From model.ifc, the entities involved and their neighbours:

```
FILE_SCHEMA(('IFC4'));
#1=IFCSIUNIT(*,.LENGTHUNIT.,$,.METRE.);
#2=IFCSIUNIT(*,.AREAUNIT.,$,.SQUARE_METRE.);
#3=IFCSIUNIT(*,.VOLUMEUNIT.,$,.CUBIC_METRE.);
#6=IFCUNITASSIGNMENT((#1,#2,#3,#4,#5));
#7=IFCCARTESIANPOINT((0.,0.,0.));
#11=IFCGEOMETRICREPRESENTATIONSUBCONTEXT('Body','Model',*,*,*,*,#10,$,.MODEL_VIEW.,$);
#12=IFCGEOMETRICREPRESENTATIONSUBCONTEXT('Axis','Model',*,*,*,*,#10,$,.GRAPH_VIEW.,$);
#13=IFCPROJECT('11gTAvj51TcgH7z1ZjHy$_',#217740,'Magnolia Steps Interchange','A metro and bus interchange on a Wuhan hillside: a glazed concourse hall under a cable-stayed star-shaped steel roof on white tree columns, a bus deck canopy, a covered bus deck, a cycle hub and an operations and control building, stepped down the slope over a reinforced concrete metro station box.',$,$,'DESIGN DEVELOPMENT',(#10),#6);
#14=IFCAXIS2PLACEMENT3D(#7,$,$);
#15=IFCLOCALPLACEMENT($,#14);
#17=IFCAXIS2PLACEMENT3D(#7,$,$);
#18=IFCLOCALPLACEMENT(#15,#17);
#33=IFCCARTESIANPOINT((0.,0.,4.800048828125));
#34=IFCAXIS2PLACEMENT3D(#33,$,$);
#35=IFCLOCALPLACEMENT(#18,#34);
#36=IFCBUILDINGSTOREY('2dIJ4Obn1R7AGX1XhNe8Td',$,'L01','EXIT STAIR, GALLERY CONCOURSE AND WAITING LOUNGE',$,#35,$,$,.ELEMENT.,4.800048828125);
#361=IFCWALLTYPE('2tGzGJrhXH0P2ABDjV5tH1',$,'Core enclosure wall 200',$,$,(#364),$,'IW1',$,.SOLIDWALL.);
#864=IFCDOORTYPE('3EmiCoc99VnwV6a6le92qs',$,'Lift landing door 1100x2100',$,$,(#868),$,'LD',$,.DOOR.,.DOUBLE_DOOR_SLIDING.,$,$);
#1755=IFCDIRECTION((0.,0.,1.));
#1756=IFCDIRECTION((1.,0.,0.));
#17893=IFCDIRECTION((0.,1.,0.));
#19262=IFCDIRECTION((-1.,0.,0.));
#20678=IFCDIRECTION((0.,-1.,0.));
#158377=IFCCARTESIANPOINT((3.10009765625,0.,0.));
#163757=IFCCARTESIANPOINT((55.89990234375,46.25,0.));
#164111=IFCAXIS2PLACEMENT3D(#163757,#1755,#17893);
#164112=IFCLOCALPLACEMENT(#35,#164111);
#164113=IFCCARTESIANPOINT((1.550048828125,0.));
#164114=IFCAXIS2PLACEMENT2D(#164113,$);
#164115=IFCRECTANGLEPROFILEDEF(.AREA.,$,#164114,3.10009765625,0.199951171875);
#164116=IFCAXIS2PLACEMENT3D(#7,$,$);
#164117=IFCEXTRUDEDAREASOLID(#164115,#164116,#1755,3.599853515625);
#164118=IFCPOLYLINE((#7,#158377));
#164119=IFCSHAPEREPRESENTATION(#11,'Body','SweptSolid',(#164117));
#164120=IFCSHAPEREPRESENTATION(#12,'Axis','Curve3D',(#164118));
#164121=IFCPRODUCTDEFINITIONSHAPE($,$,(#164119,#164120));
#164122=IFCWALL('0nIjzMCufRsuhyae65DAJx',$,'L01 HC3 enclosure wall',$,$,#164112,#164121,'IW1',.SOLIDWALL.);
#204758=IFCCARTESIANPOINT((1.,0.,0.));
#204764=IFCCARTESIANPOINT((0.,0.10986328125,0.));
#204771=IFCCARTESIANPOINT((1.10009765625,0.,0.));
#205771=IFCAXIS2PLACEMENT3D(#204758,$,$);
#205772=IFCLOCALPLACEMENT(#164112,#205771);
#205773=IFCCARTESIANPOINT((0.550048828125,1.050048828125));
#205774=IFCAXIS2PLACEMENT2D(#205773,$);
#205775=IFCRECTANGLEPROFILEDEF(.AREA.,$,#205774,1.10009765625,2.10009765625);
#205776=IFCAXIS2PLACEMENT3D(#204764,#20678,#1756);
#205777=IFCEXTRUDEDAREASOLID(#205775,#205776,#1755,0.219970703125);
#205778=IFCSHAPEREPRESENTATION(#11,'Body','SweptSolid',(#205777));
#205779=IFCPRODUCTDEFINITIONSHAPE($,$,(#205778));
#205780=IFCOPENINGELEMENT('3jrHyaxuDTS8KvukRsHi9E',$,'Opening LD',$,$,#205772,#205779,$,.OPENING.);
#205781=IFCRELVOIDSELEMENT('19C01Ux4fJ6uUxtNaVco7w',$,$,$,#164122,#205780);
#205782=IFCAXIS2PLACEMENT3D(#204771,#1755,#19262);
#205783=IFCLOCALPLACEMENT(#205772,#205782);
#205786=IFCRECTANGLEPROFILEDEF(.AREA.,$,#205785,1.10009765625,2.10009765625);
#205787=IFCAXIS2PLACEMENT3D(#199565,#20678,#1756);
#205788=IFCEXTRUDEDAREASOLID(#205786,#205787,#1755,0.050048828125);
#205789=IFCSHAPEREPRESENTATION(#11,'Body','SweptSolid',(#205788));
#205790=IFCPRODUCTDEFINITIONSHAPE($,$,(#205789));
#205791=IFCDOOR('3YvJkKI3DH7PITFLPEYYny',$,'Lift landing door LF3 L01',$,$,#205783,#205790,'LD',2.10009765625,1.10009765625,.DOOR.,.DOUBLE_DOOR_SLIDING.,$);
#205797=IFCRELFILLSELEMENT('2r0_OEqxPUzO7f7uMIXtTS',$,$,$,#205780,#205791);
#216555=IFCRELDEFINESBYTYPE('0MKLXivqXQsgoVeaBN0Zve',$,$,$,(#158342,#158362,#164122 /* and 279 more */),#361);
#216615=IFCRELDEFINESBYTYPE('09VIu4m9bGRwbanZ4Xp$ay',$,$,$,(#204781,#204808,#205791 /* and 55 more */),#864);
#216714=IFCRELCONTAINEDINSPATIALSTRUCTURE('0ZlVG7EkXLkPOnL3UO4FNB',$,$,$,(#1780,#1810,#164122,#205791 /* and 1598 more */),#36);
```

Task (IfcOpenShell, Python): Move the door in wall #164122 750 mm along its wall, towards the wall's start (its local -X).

```python
import ifcopenshell
import ifcopenshell.api.geometry
import ifcopenshell.util.placement
import ifcopenshell.util.unit

model = ifcopenshell.open("model.ifc")
unit_scale = ifcopenshell.util.unit.calculate_unit_scale(model)

door = model.by_guid("3YvJkKI3DH7PITFLPEYYny")
opening = door.FillsVoids[0].RelatingOpeningElement
wall = opening.VoidsElements[0].RelatingBuildingElement

wall_matrix = ifcopenshell.util.placement.get_local_placement(wall.ObjectPlacement)
shift = wall_matrix[:3, 0] * -0.75 / unit_scale
before = ifcopenshell.util.placement.get_local_placement(door.ObjectPlacement)[:3, 3].copy()

# The door is placed relative to its opening, so it follows when the opening moves.
matrix = ifcopenshell.util.placement.get_local_placement(opening.ObjectPlacement)
matrix[:3, 3] += shift
ifcopenshell.api.geometry.edit_object_placement(
    model, product=opening, matrix=matrix, is_si=False, should_transform_children=True
)

after = ifcopenshell.util.placement.get_local_placement(door.ObjectPlacement)[:3, 3]
print("door moved by", (after - before).round(3) + 0.0)

model.write("model-out.ifc")
```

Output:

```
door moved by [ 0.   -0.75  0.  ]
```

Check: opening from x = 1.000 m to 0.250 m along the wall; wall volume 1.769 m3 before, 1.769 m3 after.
